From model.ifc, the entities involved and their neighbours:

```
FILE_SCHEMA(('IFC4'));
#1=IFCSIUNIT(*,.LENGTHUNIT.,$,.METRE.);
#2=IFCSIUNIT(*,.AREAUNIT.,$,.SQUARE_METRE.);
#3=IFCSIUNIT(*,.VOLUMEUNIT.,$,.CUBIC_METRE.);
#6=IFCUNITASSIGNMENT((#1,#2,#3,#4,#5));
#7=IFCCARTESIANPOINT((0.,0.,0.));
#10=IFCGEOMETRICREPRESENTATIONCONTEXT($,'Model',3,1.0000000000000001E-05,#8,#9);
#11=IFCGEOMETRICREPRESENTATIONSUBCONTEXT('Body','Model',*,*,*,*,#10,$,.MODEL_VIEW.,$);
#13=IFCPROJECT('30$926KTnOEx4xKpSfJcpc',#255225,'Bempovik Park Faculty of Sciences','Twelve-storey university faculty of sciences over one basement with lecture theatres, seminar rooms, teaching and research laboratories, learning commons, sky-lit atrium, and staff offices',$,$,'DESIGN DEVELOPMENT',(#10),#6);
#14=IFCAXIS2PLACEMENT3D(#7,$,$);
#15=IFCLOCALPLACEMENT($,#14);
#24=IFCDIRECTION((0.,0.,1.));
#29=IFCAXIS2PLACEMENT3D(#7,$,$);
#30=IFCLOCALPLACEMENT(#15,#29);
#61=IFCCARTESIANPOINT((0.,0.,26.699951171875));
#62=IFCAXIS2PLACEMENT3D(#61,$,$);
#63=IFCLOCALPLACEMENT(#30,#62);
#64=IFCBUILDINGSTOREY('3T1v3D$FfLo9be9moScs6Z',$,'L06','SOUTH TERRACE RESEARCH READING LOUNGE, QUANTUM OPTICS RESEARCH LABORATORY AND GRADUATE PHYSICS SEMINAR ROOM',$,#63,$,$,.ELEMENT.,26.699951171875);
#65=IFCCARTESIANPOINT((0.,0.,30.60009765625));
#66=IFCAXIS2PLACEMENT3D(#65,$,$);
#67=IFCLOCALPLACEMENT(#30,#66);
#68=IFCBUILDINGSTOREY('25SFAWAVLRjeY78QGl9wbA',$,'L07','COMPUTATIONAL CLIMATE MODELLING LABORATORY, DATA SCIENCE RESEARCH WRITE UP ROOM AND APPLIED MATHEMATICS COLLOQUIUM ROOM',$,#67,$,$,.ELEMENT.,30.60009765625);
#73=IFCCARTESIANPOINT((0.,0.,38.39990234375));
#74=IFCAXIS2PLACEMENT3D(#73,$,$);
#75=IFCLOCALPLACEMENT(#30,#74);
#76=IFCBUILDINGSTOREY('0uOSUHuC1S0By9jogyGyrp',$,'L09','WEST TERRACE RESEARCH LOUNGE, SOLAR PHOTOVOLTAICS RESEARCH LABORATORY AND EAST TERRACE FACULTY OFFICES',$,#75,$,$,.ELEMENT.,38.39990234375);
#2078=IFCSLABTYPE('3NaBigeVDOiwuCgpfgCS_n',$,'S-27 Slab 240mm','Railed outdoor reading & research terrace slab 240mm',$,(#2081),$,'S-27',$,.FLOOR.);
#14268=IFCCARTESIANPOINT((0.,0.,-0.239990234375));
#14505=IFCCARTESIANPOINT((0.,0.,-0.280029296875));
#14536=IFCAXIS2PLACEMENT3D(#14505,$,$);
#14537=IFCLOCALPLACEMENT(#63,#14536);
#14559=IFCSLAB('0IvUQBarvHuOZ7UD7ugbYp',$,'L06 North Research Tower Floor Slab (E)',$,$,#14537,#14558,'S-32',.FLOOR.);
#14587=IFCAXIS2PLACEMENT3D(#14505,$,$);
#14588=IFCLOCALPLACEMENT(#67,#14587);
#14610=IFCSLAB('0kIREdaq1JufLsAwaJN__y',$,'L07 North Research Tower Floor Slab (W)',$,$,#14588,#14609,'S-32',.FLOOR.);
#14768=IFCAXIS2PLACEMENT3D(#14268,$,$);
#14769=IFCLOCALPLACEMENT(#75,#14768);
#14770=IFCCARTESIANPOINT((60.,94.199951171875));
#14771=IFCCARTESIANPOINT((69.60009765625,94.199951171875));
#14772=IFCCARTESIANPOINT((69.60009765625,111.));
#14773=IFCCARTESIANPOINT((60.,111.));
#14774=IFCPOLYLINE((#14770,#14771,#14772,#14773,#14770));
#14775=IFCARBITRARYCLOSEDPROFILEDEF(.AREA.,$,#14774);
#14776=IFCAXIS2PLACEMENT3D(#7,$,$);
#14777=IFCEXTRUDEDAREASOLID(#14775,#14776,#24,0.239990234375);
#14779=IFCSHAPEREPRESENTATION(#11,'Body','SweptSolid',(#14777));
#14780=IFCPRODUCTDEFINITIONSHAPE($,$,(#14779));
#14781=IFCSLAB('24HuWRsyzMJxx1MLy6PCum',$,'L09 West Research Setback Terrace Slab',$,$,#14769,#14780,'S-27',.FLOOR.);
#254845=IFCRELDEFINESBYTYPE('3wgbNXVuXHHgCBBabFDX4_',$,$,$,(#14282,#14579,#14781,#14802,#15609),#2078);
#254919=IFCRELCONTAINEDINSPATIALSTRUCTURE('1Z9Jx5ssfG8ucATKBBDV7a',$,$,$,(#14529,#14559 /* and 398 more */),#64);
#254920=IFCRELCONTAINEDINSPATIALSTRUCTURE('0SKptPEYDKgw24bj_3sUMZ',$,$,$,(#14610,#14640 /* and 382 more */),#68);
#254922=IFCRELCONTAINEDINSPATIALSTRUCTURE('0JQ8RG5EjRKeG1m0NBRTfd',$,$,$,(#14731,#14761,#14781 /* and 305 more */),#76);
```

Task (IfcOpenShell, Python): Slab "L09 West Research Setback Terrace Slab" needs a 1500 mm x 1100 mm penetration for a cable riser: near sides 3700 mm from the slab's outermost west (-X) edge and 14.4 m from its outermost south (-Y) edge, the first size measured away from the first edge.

```python
import numpy as np
import ifcopenshell
import ifcopenshell.api.feature
import ifcopenshell.api.geometry
import ifcopenshell.api.root
import ifcopenshell.geom
import ifcopenshell.util.placement
import ifcopenshell.util.representation
import ifcopenshell.util.shape
import ifcopenshell.util.unit

model = ifcopenshell.open("model.ifc")
unit_scale = ifcopenshell.util.unit.calculate_unit_scale(model)
settings = ifcopenshell.geom.settings()


def volume(element):
    """Net volume in cubic metres, openings subtracted."""
    shape = ifcopenshell.geom.create_shape(settings, element)
    return ifcopenshell.util.shape.get_volume(shape.geometry)


slab = model.by_guid("24HuWRsyzMJxx1MLy6PCum")
before = volume(slab)

# Extent in the slab's own axes, in metres. The edges named are its -X and -Y sides.
slab_shape = ifcopenshell.geom.create_shape(settings, slab)
vertices = ifcopenshell.util.shape.get_vertices(slab_shape.geometry)
x_min, y_min, bottom = vertices.min(axis=0)
top = vertices[:, 2].max()

opening = ifcopenshell.api.root.create_entity(model, ifc_class="IfcOpeningElement", name="Cable riser opening", predefined_type="OPENING")
context = ifcopenshell.util.representation.get_context(model, "Model", "Body", "MODEL_VIEW")
width, depth = 1.5, 1.1
outline = [(0.0, 0.0), (width, 0.0), (width, depth), (0.0, depth), (0.0, 0.0)]
# Overshoot both faces by 50 mm so the cut is clean.
shape = ifcopenshell.api.geometry.add_slab_representation(
    model, context=context, depth=top - bottom + 0.1, polyline=outline
)
ifcopenshell.api.geometry.assign_representation(model, product=opening, representation=shape)

matrix = ifcopenshell.util.placement.get_local_placement(slab.ObjectPlacement)
matrix[:, 3] = matrix @ np.append(np.array([x_min + 3.7, y_min + 14.4, bottom - 0.05]) / unit_scale, 1.0)
ifcopenshell.api.geometry.edit_object_placement(model, product=opening, matrix=matrix, is_si=False)
ifcopenshell.api.feature.add_feature(model, feature=opening, element=slab)

after = volume(slab)

print(f"slab volume {before:.3f} -> {after:.3f} m3")

model.write("model_rev.ifc")
```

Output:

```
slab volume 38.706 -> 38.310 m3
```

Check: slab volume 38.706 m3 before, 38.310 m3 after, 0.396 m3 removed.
